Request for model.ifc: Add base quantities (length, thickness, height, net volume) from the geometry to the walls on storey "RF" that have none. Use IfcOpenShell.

First a look at what the model holds.

```python
import ifcopenshell
import ifcopenshell.util.element
import ifcopenshell.util.unit

model = ifcopenshell.open("model.ifc")
print(model.schema)
for unit_type in ("LENGTHUNIT", "AREAUNIT", "VOLUMEUNIT"):
    print(unit_type, ifcopenshell.util.unit.calculate_unit_scale(model, unit_type))
storey = next(s for s in model.by_type("IfcBuildingStorey") if s.Name == "RF")
walls = [e for e in ifcopenshell.util.element.get_decomposition(storey) if e.is_a("IfcWall")]
for e in sorted(walls, key=lambda e: e.id()):
    print(e.id(), e.is_a(), e.Name, list(ifcopenshell.util.element.get_psets(e, qtos_only=True)), sep=" | ")
```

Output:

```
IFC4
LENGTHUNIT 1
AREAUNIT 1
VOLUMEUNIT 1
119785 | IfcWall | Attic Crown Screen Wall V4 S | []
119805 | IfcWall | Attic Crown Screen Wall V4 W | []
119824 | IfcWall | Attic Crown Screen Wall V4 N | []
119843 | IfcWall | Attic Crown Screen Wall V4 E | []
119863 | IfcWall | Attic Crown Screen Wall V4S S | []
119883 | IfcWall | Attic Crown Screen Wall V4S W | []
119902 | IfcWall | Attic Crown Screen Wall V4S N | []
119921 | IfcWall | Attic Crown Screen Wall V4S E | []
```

```python
import ifcopenshell
import ifcopenshell.api.pset
import ifcopenshell.geom
import ifcopenshell.util.element
import ifcopenshell.util.shape
import ifcopenshell.util.unit

model = ifcopenshell.open("model.ifc")
unit_scale = ifcopenshell.util.unit.calculate_unit_scale(model)
volume_scale = ifcopenshell.util.unit.calculate_unit_scale(model, "VOLUMEUNIT")
settings = ifcopenshell.geom.settings()

storey = next(s for s in model.by_type("IfcBuildingStorey") if s.Name == "RF")
walls = [e for e in ifcopenshell.util.element.get_decomposition(storey) if e.is_a("IfcWall")]

for e in sorted(walls, key=lambda e: e.id()):
    if ifcopenshell.util.element.get_psets(e, qtos_only=True, should_inherit=False):
        continue
    # Geometry comes back in metres, in the element's own axes.
    shape = ifcopenshell.geom.create_shape(settings, e)
    values = {
        "Length": ifcopenshell.util.shape.get_x(shape.geometry) / unit_scale,
        "Width": ifcopenshell.util.shape.get_y(shape.geometry) / unit_scale,
        "Height": ifcopenshell.util.shape.get_z(shape.geometry) / unit_scale,
        "NetVolume": ifcopenshell.util.shape.get_volume(shape.geometry) / volume_scale,
    }
    qto = ifcopenshell.api.pset.add_qto(model, product=e, name="Qto_WallBaseQuantities")
    ifcopenshell.api.pset.edit_qto(model, qto=qto, properties=values)
    print(e.id(), {k: round(v, 3) for k, v in values.items()})

model.write("model-out.ifc")
```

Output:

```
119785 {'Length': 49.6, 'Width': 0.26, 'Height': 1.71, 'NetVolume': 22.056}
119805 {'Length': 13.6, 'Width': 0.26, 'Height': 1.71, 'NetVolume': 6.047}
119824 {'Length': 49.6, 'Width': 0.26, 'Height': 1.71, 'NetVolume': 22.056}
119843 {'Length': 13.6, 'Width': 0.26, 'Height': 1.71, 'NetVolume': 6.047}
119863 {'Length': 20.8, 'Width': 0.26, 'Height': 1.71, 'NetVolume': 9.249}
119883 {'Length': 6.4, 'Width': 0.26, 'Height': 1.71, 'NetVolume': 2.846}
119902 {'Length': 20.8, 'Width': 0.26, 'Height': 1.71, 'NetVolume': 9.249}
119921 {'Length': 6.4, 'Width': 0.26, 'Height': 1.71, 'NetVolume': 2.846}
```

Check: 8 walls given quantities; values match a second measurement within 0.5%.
